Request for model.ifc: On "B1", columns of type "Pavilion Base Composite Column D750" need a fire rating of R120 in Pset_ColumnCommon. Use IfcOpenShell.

First a look at what the model holds.

```python
import ifcopenshell
import ifcopenshell.util.element

model = ifcopenshell.open("model.ifc")
print(model.schema)
storey = next(s for s in model.by_type("IfcBuildingStorey") if s.Name == "B1")
columns = [e for e in ifcopenshell.util.element.get_decomposition(storey) if e.is_a("IfcColumn")]
seen = {}
for e in columns:
    element_type = ifcopenshell.util.element.get_type(e)
    key = (element_type.Name if element_type != e and element_type else None, ifcopenshell.util.element.get_pset(e, "Pset_ColumnCommon", "FireRating"))
    seen[key] = seen.get(key, 0) + 1
for (name, value), count in sorted(seen.items(), key=str):
    print(count, "x", name, "|", value)
```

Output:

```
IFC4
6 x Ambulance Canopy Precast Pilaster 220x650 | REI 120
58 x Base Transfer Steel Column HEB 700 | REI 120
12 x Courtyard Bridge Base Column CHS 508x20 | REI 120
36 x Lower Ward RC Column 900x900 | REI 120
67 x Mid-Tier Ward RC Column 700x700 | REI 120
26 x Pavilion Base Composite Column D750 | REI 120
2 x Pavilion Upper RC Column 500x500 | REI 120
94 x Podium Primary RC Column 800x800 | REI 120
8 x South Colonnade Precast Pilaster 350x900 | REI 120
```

```python
import ifcopenshell
import ifcopenshell.api.pset
import ifcopenshell.util.element

model = ifcopenshell.open("model.ifc")

storey = next(s for s in model.by_type("IfcBuildingStorey") if s.Name == "B1")
columns = [e for e in ifcopenshell.util.element.get_decomposition(storey) if e.is_a("IfcColumn")]

count = 0
for e in columns:
    element_type = ifcopenshell.util.element.get_type(e)
    if element_type in (None, e) or element_type.Name != "Pavilion Base Composite Column D750":
        continue
    # add_pset returns the element's existing set when there is one.
    pset = ifcopenshell.api.pset.add_pset(model, product=e, name="Pset_ColumnCommon")
    ifcopenshell.api.pset.edit_pset(model, pset=pset, properties={"FireRating": "R120"})
    count += 1

print(count, "columns updated")

model.write("model-out.ifc")
```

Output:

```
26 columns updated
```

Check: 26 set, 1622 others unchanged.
